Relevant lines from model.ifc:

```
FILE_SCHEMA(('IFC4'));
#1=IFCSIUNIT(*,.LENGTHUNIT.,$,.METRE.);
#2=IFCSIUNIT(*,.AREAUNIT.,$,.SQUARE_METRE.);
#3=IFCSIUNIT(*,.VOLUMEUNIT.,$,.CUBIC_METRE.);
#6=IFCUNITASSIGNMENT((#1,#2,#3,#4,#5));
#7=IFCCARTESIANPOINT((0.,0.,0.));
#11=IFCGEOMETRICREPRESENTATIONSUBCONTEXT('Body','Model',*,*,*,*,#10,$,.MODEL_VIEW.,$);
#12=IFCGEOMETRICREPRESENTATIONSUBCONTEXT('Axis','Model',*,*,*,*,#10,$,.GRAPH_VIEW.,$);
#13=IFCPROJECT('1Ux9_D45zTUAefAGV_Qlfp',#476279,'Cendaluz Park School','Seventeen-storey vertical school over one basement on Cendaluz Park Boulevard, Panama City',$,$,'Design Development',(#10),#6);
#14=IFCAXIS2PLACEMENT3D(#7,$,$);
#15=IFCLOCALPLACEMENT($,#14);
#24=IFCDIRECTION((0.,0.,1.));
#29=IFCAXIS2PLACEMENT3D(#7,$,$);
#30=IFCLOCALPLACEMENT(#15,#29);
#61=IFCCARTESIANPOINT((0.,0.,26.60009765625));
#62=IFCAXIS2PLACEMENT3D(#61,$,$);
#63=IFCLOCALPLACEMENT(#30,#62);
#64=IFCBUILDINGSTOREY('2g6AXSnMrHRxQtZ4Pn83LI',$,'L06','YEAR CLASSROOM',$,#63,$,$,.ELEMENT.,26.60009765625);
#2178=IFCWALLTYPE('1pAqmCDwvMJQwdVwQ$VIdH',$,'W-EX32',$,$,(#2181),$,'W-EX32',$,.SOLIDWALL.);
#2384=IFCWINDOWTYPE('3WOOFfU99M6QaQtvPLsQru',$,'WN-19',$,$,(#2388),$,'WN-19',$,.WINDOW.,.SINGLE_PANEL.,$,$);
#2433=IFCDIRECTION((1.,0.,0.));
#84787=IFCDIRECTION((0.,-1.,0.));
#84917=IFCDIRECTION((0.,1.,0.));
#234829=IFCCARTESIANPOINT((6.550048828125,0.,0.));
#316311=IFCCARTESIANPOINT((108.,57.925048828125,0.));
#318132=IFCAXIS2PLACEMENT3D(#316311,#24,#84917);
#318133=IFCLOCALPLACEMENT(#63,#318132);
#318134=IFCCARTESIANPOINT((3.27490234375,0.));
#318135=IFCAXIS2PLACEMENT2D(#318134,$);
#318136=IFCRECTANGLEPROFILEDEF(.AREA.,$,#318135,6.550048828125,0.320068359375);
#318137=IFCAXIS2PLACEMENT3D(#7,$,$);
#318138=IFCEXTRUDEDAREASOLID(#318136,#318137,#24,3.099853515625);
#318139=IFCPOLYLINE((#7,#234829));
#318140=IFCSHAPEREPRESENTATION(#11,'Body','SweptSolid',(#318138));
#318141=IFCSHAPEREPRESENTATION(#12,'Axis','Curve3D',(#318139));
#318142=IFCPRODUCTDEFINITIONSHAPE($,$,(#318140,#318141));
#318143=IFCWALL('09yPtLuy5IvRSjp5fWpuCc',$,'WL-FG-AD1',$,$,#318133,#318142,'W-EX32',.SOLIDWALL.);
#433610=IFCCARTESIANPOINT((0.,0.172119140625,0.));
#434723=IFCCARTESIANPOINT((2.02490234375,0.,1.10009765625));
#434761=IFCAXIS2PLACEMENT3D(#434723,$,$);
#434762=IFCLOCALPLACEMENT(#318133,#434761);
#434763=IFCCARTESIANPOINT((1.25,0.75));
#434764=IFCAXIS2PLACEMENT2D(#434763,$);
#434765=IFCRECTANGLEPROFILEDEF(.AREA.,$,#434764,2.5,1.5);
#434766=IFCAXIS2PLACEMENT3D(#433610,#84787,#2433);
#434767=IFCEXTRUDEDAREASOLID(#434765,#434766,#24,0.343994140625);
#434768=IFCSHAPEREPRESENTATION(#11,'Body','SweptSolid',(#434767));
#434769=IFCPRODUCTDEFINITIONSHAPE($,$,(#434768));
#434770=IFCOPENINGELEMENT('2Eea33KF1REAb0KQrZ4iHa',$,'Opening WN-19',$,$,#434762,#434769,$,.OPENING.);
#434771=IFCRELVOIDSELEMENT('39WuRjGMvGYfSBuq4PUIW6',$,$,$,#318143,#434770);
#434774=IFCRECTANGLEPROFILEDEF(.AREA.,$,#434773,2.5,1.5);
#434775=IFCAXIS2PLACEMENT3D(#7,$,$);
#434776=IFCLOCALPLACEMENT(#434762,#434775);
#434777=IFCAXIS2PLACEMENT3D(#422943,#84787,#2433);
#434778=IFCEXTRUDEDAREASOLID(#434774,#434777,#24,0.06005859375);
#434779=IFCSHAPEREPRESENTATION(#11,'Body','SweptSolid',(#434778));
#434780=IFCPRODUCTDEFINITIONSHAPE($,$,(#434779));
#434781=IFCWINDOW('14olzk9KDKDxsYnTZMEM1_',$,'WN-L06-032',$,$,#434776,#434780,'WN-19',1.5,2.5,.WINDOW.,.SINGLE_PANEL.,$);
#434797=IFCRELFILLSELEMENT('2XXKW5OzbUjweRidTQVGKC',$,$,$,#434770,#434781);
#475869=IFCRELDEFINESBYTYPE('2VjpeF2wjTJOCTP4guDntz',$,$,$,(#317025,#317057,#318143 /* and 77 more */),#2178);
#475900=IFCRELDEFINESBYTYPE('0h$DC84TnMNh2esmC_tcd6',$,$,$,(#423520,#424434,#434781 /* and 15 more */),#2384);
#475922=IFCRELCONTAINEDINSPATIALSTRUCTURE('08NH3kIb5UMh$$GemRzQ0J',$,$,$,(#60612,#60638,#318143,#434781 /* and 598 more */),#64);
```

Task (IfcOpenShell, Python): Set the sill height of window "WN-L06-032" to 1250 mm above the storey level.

```python
import numpy as np
import ifcopenshell
import ifcopenshell.api.geometry
import ifcopenshell.geom
import ifcopenshell.util.element
import ifcopenshell.util.placement
import ifcopenshell.util.shape
import ifcopenshell.util.unit

model = ifcopenshell.open("model.ifc")
unit_scale = ifcopenshell.util.unit.calculate_unit_scale(model)

window = model.by_guid("14olzk9KDKDxsYnTZMEM1_")
opening = window.FillsVoids[0].RelatingOpeningElement
storey = ifcopenshell.util.element.get_container(window, ifc_class="IfcBuildingStorey")
level = ifcopenshell.util.placement.get_local_placement(storey.ObjectPlacement)[2, 3]

# The opening's origin need not be at the sill, so measure its lowest point.
shape = ifcopenshell.geom.create_shape(ifcopenshell.geom.settings(), opening)
bottom = ifcopenshell.util.shape.get_shape_bottom_elevation(shape, shape.geometry) / unit_scale
dz = level + 1.25 - bottom

shift = np.array([0.0, 0.0, dz])
# The window is placed relative to its opening, so it follows when the opening moves.
matrix = ifcopenshell.util.placement.get_local_placement(opening.ObjectPlacement)
matrix[:3, 3] += shift
ifcopenshell.api.geometry.edit_object_placement(
    model, product=opening, matrix=matrix, is_si=False, should_transform_children=True
)

print(f"moved by {dz * unit_scale:+.3f} m")

model.write("model_updated.ifc")
```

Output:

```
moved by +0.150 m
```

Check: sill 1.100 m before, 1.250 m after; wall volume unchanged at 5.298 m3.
